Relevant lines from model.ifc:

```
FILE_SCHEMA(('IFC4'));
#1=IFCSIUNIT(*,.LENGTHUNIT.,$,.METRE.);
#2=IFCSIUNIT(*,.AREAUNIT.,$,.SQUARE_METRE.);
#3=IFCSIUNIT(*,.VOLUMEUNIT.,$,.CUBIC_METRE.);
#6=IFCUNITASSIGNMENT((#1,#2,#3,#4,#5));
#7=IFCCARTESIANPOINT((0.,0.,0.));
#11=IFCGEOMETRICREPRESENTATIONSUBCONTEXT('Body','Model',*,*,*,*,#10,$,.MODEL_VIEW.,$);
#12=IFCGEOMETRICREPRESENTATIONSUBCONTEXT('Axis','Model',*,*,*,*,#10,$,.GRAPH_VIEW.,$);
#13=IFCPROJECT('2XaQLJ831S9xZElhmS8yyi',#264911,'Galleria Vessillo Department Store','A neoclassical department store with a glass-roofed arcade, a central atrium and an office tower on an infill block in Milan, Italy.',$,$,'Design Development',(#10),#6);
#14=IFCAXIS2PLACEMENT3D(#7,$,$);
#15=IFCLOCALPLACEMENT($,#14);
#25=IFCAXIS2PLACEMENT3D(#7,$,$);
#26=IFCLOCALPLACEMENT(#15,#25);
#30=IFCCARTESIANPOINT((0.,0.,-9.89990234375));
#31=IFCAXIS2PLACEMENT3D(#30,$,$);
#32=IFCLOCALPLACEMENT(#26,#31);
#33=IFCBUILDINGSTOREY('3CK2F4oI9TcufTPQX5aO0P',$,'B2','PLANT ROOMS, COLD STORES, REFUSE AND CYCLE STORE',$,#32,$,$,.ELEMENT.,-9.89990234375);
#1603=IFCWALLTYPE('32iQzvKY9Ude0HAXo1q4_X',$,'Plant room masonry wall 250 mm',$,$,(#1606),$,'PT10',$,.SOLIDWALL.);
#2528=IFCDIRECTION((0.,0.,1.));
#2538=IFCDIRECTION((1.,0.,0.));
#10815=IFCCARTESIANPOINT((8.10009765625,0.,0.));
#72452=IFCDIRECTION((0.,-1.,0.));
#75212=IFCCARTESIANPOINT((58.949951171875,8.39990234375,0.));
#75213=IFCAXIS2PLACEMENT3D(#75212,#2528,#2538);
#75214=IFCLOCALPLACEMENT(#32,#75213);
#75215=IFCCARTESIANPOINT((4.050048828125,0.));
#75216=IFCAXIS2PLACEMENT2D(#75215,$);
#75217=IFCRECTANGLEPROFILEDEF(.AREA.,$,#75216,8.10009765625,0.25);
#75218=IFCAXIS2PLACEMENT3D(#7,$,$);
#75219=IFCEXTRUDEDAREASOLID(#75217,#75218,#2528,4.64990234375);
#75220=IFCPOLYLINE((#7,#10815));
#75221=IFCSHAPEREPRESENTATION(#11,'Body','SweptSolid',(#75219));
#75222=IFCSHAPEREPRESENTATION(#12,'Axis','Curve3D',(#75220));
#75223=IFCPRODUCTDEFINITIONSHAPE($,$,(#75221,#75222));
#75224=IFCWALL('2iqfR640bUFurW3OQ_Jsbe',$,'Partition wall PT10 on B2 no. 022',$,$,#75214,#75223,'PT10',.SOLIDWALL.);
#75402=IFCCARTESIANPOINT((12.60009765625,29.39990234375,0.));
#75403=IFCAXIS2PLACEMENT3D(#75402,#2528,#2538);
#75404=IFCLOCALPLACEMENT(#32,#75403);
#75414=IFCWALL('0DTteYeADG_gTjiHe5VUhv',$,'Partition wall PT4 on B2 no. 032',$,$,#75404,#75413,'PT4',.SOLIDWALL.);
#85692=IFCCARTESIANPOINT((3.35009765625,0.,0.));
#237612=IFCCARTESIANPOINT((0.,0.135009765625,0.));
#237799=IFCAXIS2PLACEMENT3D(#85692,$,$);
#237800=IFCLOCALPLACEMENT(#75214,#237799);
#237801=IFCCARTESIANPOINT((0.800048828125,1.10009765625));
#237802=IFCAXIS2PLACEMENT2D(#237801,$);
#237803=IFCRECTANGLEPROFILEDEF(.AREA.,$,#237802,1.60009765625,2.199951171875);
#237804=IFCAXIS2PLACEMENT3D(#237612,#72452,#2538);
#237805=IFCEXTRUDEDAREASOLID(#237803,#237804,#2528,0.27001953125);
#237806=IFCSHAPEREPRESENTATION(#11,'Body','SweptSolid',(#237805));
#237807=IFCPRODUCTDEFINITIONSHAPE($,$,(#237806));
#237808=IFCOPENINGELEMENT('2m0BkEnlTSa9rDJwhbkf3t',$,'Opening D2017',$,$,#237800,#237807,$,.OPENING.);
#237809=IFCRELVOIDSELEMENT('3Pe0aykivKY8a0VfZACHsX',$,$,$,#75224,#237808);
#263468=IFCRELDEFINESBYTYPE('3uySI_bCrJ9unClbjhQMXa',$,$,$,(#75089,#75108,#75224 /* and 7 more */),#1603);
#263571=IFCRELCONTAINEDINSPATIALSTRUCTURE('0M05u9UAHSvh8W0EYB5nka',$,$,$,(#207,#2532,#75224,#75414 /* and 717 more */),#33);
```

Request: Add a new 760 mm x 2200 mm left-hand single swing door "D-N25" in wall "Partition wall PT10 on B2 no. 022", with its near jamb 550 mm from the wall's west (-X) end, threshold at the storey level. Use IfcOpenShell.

```python
import numpy as np
import ifcopenshell
import ifcopenshell.api.feature
import ifcopenshell.api.geometry
import ifcopenshell.api.root
import ifcopenshell.api.spatial
import ifcopenshell.geom
import ifcopenshell.util.element
import ifcopenshell.util.placement
import ifcopenshell.util.representation
import ifcopenshell.util.shape
import ifcopenshell.util.unit

model = ifcopenshell.open("model.ifc")
unit_scale = ifcopenshell.util.unit.calculate_unit_scale(model)
settings = ifcopenshell.geom.settings()


def volume(element):
    """Net volume in cubic metres, openings subtracted."""
    shape = ifcopenshell.geom.create_shape(settings, element)
    return ifcopenshell.util.shape.get_volume(shape.geometry)


wall = model.by_guid("2iqfR640bUFurW3OQ_Jsbe")
storey = ifcopenshell.util.element.get_container(wall, ifc_class="IfcBuildingStorey")
context = ifcopenshell.util.representation.get_context(model, "Model", "Body", "MODEL_VIEW")
before = volume(wall)

width, height, from_end, sill = 0.76, 2.2, 0.55, 0.0  # metres

# The wall runs along its own X axis, and the end named is its -X end.
wall_shape = ifcopenshell.geom.create_shape(settings, wall)
x, y, z = ifcopenshell.util.shape.get_vertices(wall_shape.geometry).T
start = x.min() + from_end
face, thickness = float(y.min()), float(y.max() - y.min())
wall_matrix = ifcopenshell.util.placement.get_local_placement(wall.ObjectPlacement)
level = ifcopenshell.util.placement.get_local_placement(storey.ObjectPlacement)[2, 3]


def in_wall(x, y):
    """Placement at x, y metres in the wall's axes, at sill height."""
    matrix = wall_matrix.copy()
    matrix[:, 3] = wall_matrix @ np.array([x / unit_scale, y / unit_scale, 0.0, 1.0])
    matrix[2, 3] = level + sill / unit_scale
    return matrix


# Opening: a box that overshoots both wall faces by 50 mm.
opening = ifcopenshell.api.root.create_entity(model, ifc_class="IfcOpeningElement", predefined_type="OPENING")
box = ifcopenshell.api.geometry.add_wall_representation(
    model, context=context, length=width, height=height, thickness=thickness + 0.1
)
ifcopenshell.api.geometry.assign_representation(model, product=opening, representation=box)
ifcopenshell.api.geometry.edit_object_placement(model, product=opening, matrix=in_wall(start, face - 0.05), is_si=False)
ifcopenshell.api.feature.add_feature(model, feature=opening, element=wall)

door = ifcopenshell.api.root.create_entity(model, ifc_class="IfcDoor", name="D-N25", predefined_type="DOOR")
door.OverallWidth, door.OverallHeight = width / unit_scale, height / unit_scale
door.OperationType = "SINGLE_SWING_LEFT"
body = ifcopenshell.api.geometry.add_door_representation(
    model,
    context=context,
    overall_width=door.OverallWidth,
    overall_height=door.OverallHeight,
    operation_type="SINGLE_SWING_LEFT",
    lining_properties={"LiningDepth": thickness / unit_scale, "ThresholdDepth": thickness / unit_scale},
)
ifcopenshell.api.geometry.assign_representation(model, product=door, representation=body)
ifcopenshell.api.spatial.assign_container(model, products=[door], relating_structure=storey)
ifcopenshell.api.feature.add_filling(model, opening=opening, element=door)

# The lining spans the wall, so the door starts at the wall face.
ifcopenshell.api.geometry.edit_object_placement(model, product=door, matrix=in_wall(start, face), is_si=False)

after = volume(wall)

print(f"wall volume {before:.3f} -> {after:.3f} m3")

model.write("model_rev.ifc")
```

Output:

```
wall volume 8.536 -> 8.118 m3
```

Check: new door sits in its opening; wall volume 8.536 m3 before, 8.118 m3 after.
